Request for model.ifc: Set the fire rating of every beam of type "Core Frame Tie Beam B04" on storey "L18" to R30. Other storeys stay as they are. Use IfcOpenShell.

First a look at what the model holds.

```python
import ifcopenshell
import ifcopenshell.util.element

model = ifcopenshell.open("model.ifc")
print(model.schema)
storey = next(s for s in model.by_type("IfcBuildingStorey") if s.Name == "L18")
beams = [e for e in ifcopenshell.util.element.get_decomposition(storey) if e.is_a("IfcBeam")]
seen = {}
for e in beams:
    element_type = ifcopenshell.util.element.get_type(e)
    key = (element_type.Name if element_type != e and element_type else None, ifcopenshell.util.element.get_pset(e, "Pset_BeamCommon", "FireRating"))
    seen[key] = seen.get(key, 0) + 1
for (name, value), count in sorted(seen.items(), key=str):
    print(count, "x", name, "|", value)
```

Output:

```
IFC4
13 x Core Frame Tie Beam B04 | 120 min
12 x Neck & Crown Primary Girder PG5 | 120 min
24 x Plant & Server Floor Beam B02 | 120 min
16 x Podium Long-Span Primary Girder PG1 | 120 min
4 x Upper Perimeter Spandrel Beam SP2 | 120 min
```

```python
import ifcopenshell
import ifcopenshell.api.pset
import ifcopenshell.util.element

model = ifcopenshell.open("model.ifc")

storey = next(s for s in model.by_type("IfcBuildingStorey") if s.Name == "L18")
beams = [e for e in ifcopenshell.util.element.get_decomposition(storey) if e.is_a("IfcBeam")]

count = 0
for e in beams:
    element_type = ifcopenshell.util.element.get_type(e)
    if element_type in (None, e) or element_type.Name != "Core Frame Tie Beam B04":
        continue
    found = ifcopenshell.util.element.get_pset(e, "Pset_BeamCommon", should_inherit=False)
    if found:
        pset = model.by_id(found["id"])
        if len(ifcopenshell.util.element.get_elements_by_pset(pset)) > 1:
            pset = ifcopenshell.api.pset.unshare_pset(model, products=[e], pset=pset)[0]
    else:
        pset = ifcopenshell.api.pset.add_pset(model, product=e, name="Pset_BeamCommon")
    ifcopenshell.api.pset.edit_pset(model, pset=pset, properties={"FireRating": "R30"})
    count += 1

print(count, "beams updated")

model.write("model_edited.ifc")
```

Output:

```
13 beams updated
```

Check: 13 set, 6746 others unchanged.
